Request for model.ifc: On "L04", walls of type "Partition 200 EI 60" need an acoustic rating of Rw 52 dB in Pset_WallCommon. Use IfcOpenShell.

First a look at what the model holds.

```python
import ifcopenshell
import ifcopenshell.util.element

model = ifcopenshell.open("model.ifc")
print(model.schema)
storey = next(s for s in model.by_type("IfcBuildingStorey") if s.Name == "L04")
walls = [e for e in ifcopenshell.util.element.get_decomposition(storey) if e.is_a("IfcWall")]
seen = {}
for e in walls:
    element_type = ifcopenshell.util.element.get_type(e)
    key = (element_type.Name if element_type != e and element_type else None, ifcopenshell.util.element.get_pset(e, "Pset_WallCommon", "AcousticRating"))
    seen[key] = seen.get(key, 0) + 1
for (name, value), count in sorted(seen.items(), key=str):
    print(count, "x", name, "|", value)
```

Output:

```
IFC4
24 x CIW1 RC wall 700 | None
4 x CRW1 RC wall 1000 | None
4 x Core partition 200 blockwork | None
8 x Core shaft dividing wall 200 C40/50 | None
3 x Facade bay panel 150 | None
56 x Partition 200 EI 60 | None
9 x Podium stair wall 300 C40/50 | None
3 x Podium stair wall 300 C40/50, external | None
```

```python
import ifcopenshell
import ifcopenshell.api.pset
import ifcopenshell.util.element

model = ifcopenshell.open("model.ifc")

storey = next(s for s in model.by_type("IfcBuildingStorey") if s.Name == "L04")
walls = [e for e in ifcopenshell.util.element.get_decomposition(storey) if e.is_a("IfcWall")]

count = 0
for e in walls:
    element_type = ifcopenshell.util.element.get_type(e)
    if element_type in (None, e) or element_type.Name != "Partition 200 EI 60":
        continue
    found = ifcopenshell.util.element.get_pset(e, "Pset_WallCommon", should_inherit=False)
    if found:
        pset = model.by_id(found["id"])
        if len(ifcopenshell.util.element.get_elements_by_pset(pset)) > 1:
            pset = ifcopenshell.api.pset.unshare_pset(model, products=[e], pset=pset)[0]
    else:
        pset = ifcopenshell.api.pset.add_pset(model, product=e, name="Pset_WallCommon")
    ifcopenshell.api.pset.edit_pset(model, pset=pset, properties={"AcousticRating": "Rw 52 dB"})
    count += 1

print(count, "walls updated")

model.write("model_updated.ifc")
```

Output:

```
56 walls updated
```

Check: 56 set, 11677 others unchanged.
